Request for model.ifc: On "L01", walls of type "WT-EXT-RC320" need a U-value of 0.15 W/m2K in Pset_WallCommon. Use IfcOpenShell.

First a look at what the model holds.

```python
import ifcopenshell
import ifcopenshell.util.element

model = ifcopenshell.open("model.ifc")
print(model.schema)
storey = next(s for s in model.by_type("IfcBuildingStorey") if s.Name == "L01")
walls = [e for e in ifcopenshell.util.element.get_decomposition(storey) if e.is_a("IfcWall")]
seen = {}
for e in walls:
    element_type = ifcopenshell.util.element.get_type(e)
    key = (element_type.Name if element_type != e and element_type else None, ifcopenshell.util.element.get_pset(e, "Pset_WallCommon", "ThermalTransmittance"))
    seen[key] = seen.get(key, 0) + 1
for (name, value), count in sorted(seen.items(), key=str):
    print(count, "x", name, "|", value)
```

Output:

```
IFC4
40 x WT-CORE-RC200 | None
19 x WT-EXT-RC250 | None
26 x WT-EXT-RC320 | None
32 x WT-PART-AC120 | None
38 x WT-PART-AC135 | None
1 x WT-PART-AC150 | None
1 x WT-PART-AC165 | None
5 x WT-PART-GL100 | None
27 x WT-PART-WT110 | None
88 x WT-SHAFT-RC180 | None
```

```python
import ifcopenshell
import ifcopenshell.api.pset
import ifcopenshell.util.element

model = ifcopenshell.open("model.ifc")

storey = next(s for s in model.by_type("IfcBuildingStorey") if s.Name == "L01")
walls = [e for e in ifcopenshell.util.element.get_decomposition(storey) if e.is_a("IfcWall")]

count = 0
for e in walls:
    element_type = ifcopenshell.util.element.get_type(e)
    if element_type in (None, e) or element_type.Name != "WT-EXT-RC320":
        continue
    # add_pset returns the element's existing set when there is one.
    pset = ifcopenshell.api.pset.add_pset(model, product=e, name="Pset_WallCommon")
    ifcopenshell.api.pset.edit_pset(model, pset=pset, properties={"ThermalTransmittance": 0.15})
    count += 1

print(count, "walls updated")

model.write("model_updated.ifc")
```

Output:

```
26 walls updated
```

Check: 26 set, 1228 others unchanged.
